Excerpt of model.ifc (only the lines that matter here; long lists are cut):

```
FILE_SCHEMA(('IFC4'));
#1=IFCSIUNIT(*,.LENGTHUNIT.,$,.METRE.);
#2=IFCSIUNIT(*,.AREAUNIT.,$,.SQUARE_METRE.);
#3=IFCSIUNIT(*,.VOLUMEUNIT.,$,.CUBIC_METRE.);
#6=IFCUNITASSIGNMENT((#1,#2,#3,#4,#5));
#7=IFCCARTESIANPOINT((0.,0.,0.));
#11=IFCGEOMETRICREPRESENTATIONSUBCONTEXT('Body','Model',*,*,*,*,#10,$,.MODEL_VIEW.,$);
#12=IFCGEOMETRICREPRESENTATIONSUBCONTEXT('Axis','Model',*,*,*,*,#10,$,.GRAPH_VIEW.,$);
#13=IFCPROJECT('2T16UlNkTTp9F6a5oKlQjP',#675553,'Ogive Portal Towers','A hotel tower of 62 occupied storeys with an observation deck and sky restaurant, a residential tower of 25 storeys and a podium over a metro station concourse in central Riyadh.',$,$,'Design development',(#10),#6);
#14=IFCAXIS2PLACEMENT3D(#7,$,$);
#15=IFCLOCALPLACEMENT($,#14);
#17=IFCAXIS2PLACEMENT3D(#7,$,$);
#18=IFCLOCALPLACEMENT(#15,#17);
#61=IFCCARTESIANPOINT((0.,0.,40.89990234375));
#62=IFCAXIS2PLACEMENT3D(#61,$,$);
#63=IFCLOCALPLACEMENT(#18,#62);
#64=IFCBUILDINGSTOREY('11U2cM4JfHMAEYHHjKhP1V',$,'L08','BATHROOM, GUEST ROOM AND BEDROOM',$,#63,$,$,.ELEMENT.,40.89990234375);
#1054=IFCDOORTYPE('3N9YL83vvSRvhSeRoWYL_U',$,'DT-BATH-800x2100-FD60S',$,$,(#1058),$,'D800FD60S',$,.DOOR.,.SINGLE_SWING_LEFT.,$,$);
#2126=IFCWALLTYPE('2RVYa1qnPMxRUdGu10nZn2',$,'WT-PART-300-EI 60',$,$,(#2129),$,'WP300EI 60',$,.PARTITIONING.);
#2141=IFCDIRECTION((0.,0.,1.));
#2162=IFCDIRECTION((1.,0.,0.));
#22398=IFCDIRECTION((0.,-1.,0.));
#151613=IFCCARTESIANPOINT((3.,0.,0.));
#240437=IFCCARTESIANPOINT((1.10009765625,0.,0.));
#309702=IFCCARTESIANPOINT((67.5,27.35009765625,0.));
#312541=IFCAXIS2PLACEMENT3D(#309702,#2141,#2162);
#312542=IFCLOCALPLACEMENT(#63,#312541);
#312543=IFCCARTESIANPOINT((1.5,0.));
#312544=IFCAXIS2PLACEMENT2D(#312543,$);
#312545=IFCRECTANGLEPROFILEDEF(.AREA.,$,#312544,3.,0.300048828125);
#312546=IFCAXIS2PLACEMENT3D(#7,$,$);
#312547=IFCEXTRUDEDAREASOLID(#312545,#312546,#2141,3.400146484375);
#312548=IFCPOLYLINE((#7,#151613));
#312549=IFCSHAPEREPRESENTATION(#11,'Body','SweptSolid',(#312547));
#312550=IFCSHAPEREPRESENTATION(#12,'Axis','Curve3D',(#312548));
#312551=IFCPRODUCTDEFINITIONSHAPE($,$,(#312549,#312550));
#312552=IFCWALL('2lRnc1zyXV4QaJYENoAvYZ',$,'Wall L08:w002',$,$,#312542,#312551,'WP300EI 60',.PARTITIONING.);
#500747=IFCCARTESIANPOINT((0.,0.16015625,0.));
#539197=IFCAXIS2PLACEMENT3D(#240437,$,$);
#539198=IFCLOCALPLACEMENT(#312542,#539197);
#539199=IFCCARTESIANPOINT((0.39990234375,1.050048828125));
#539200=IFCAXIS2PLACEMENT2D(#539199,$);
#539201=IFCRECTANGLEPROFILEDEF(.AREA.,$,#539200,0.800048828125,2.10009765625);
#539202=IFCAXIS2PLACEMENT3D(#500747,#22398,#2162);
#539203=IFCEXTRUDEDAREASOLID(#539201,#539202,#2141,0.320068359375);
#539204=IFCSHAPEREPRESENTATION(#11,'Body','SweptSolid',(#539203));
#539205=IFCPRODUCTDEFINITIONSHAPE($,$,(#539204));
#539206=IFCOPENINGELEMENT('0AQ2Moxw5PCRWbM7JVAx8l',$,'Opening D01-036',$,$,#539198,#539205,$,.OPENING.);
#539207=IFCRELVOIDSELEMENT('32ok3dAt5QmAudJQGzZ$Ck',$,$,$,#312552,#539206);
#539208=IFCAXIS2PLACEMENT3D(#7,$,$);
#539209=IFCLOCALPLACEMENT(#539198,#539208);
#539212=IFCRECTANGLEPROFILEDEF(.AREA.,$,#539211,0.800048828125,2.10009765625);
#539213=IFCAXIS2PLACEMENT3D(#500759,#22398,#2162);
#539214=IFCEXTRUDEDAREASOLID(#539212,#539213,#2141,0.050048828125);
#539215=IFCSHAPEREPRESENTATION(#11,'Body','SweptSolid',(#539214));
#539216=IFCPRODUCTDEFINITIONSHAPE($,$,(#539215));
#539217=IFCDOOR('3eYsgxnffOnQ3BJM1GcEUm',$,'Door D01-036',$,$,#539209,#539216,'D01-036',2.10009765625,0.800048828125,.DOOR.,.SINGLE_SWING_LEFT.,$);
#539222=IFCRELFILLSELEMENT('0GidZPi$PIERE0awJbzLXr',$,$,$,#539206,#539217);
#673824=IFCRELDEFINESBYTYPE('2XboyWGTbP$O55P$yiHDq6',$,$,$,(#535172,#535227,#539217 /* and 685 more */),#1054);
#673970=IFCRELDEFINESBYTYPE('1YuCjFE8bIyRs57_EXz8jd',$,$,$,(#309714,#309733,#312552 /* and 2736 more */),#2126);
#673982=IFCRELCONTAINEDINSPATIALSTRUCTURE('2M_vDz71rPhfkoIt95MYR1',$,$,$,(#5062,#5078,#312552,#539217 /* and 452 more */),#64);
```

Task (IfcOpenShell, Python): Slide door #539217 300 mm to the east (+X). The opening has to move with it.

```python
import ifcopenshell
import ifcopenshell.api.geometry
import ifcopenshell.util.placement

model = ifcopenshell.open("model.ifc")

door = model.by_guid("3eYsgxnffOnQ3BJM1GcEUm")
opening = door.FillsVoids[0].RelatingOpeningElement
wall = opening.VoidsElements[0].RelatingBuildingElement

wall_matrix = ifcopenshell.util.placement.get_local_placement(wall.ObjectPlacement)
shift = wall_matrix[:3, 0] * 0.3
before = ifcopenshell.util.placement.get_local_placement(door.ObjectPlacement)[:3, 3].copy()

# The door is placed relative to its opening, so it follows when the opening moves.
matrix = ifcopenshell.util.placement.get_local_placement(opening.ObjectPlacement)
matrix[:3, 3] += shift
ifcopenshell.api.geometry.edit_object_placement(
    model, product=opening, matrix=matrix, is_si=False, should_transform_children=True
)

after = ifcopenshell.util.placement.get_local_placement(door.ObjectPlacement)[:3, 3]
print("door moved by", (after - before).round(3) + 0.0)

model.write("model-out.ifc")
```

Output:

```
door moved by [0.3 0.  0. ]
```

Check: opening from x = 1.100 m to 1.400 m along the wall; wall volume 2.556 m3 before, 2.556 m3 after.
